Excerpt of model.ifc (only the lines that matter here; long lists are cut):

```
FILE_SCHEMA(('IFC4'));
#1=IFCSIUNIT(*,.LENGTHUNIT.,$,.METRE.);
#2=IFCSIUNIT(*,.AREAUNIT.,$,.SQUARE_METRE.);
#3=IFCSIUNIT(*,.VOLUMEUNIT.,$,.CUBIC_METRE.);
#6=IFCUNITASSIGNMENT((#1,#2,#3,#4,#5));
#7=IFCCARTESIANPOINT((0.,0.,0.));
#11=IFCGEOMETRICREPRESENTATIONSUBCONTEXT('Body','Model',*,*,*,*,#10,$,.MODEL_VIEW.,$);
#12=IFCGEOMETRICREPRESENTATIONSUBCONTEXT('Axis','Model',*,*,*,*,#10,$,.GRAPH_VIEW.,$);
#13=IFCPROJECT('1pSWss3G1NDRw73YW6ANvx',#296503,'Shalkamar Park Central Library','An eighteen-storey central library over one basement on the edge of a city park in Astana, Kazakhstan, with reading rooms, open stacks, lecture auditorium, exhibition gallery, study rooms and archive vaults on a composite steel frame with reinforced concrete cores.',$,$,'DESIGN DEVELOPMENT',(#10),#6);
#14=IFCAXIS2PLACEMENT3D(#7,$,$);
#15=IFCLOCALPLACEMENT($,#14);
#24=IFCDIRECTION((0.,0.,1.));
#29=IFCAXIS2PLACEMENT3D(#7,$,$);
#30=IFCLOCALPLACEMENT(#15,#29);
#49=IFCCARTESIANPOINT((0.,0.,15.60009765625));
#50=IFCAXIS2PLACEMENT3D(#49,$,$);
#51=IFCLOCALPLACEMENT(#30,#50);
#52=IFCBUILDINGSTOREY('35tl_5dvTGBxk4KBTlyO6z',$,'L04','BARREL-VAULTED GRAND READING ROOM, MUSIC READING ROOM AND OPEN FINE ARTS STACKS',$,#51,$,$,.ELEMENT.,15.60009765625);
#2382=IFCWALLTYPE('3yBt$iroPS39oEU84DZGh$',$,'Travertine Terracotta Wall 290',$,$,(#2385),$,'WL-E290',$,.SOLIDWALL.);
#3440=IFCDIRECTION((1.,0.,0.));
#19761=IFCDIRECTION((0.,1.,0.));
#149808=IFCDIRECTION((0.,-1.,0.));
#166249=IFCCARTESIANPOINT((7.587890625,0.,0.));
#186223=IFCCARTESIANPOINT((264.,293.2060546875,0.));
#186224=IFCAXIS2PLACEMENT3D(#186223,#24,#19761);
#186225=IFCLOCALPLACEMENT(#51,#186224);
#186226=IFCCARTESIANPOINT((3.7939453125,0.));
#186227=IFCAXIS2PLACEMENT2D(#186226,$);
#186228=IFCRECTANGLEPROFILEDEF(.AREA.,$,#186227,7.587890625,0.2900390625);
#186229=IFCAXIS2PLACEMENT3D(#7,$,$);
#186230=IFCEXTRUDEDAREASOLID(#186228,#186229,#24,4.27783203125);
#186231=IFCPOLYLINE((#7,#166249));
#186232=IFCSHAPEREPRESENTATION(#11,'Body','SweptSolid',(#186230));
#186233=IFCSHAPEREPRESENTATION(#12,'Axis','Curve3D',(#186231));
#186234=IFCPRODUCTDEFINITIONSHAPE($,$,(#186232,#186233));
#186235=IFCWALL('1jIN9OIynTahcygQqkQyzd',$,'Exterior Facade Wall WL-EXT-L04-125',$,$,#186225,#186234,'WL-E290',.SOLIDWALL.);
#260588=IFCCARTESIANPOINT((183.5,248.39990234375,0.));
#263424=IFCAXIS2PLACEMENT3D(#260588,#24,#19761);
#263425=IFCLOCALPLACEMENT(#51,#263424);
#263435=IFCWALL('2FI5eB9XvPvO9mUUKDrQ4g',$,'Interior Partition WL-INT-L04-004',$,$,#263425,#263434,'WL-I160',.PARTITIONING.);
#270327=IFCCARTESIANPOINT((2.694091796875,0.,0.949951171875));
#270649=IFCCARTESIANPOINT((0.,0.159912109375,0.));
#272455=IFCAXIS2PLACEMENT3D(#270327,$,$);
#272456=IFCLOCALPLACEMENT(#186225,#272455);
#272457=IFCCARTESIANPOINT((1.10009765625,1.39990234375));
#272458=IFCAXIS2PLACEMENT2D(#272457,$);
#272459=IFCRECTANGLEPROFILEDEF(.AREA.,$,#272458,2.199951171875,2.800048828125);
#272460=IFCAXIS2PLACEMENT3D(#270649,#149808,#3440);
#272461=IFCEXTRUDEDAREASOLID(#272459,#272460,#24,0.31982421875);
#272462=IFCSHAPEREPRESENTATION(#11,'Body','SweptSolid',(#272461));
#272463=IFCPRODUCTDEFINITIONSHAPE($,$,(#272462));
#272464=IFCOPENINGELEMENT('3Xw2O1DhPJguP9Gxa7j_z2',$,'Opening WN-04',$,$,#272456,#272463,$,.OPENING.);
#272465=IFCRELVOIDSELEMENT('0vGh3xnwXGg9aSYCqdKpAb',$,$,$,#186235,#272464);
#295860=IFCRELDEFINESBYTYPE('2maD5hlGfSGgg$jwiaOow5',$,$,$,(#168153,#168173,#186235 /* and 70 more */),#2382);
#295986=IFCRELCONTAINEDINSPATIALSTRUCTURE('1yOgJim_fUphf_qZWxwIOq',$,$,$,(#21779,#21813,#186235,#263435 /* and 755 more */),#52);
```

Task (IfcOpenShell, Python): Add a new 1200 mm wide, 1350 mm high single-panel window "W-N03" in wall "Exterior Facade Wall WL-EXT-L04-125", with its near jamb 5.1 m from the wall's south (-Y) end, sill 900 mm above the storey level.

```python
import numpy as np
import ifcopenshell
import ifcopenshell.api.feature
import ifcopenshell.api.geometry
import ifcopenshell.api.root
import ifcopenshell.api.spatial
import ifcopenshell.geom
import ifcopenshell.util.element
import ifcopenshell.util.placement
import ifcopenshell.util.representation
import ifcopenshell.util.shape
import ifcopenshell.util.unit

model = ifcopenshell.open("model.ifc")
unit_scale = ifcopenshell.util.unit.calculate_unit_scale(model)
settings = ifcopenshell.geom.settings()


def volume(element):
    """Net volume in cubic metres, openings subtracted."""
    shape = ifcopenshell.geom.create_shape(settings, element)
    return ifcopenshell.util.shape.get_volume(shape.geometry)


wall = model.by_id(186235)
storey = ifcopenshell.util.element.get_container(wall, ifc_class="IfcBuildingStorey")
context = ifcopenshell.util.representation.get_context(model, "Model", "Body", "MODEL_VIEW")
before = volume(wall)

width, height, from_end, sill = 1.2, 1.35, 5.1, 0.9  # metres

# The wall runs along its own X axis, and the end named is its -X end.
wall_shape = ifcopenshell.geom.create_shape(settings, wall)
x, y, z = ifcopenshell.util.shape.get_vertices(wall_shape.geometry).T
start = x.min() + from_end
face, thickness = float(y.min()), float(y.max() - y.min())
wall_matrix = ifcopenshell.util.placement.get_local_placement(wall.ObjectPlacement)
level = ifcopenshell.util.placement.get_local_placement(storey.ObjectPlacement)[2, 3]


def in_wall(x, y):
    """Placement at x, y metres in the wall's axes, at sill height."""
    matrix = wall_matrix.copy()
    matrix[:, 3] = wall_matrix @ np.array([x / unit_scale, y / unit_scale, 0.0, 1.0])
    matrix[2, 3] = level + sill / unit_scale
    return matrix


# Opening: a box that overshoots both wall faces by 50 mm.
opening = ifcopenshell.api.root.create_entity(model, ifc_class="IfcOpeningElement", predefined_type="OPENING")
box = ifcopenshell.api.geometry.add_wall_representation(
    model, context=context, length=width, height=height, thickness=thickness + 0.1
)
ifcopenshell.api.geometry.assign_representation(model, product=opening, representation=box)
ifcopenshell.api.geometry.edit_object_placement(model, product=opening, matrix=in_wall(start, face - 0.05), is_si=False)
ifcopenshell.api.feature.add_feature(model, feature=opening, element=wall)

window = ifcopenshell.api.root.create_entity(model, ifc_class="IfcWindow", name="W-N03", predefined_type="WINDOW")
window.OverallWidth, window.OverallHeight = width / unit_scale, height / unit_scale
window.PartitioningType = "SINGLE_PANEL"
body = ifcopenshell.api.geometry.add_window_representation(
    model,
    context=context,
    overall_width=window.OverallWidth,
    overall_height=window.OverallHeight,
    partition_type="SINGLE_PANEL",
)
ifcopenshell.api.geometry.assign_representation(model, product=window, representation=body)
ifcopenshell.api.spatial.assign_container(model, products=[window], relating_structure=storey)
ifcopenshell.api.feature.add_filling(model, opening=opening, element=window)

# Centre the window in the wall's thickness.
ifcopenshell.api.geometry.edit_object_placement(model, product=window, matrix=in_wall(start, face), is_si=False)
window_shape = ifcopenshell.geom.create_shape(settings, window)
depth = ifcopenshell.util.shape.get_vertices(window_shape.geometry)[:, 1]
offset = face + thickness / 2 - (depth.min() + depth.max()) / 2
ifcopenshell.api.geometry.edit_object_placement(model, product=window, matrix=in_wall(start, offset), is_si=False)

after = volume(wall)

print(f"wall volume {before:.3f} -> {after:.3f} m3")

model.write("model-out.ifc")
```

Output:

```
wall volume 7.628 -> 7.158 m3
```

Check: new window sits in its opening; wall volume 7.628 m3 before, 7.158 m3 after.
